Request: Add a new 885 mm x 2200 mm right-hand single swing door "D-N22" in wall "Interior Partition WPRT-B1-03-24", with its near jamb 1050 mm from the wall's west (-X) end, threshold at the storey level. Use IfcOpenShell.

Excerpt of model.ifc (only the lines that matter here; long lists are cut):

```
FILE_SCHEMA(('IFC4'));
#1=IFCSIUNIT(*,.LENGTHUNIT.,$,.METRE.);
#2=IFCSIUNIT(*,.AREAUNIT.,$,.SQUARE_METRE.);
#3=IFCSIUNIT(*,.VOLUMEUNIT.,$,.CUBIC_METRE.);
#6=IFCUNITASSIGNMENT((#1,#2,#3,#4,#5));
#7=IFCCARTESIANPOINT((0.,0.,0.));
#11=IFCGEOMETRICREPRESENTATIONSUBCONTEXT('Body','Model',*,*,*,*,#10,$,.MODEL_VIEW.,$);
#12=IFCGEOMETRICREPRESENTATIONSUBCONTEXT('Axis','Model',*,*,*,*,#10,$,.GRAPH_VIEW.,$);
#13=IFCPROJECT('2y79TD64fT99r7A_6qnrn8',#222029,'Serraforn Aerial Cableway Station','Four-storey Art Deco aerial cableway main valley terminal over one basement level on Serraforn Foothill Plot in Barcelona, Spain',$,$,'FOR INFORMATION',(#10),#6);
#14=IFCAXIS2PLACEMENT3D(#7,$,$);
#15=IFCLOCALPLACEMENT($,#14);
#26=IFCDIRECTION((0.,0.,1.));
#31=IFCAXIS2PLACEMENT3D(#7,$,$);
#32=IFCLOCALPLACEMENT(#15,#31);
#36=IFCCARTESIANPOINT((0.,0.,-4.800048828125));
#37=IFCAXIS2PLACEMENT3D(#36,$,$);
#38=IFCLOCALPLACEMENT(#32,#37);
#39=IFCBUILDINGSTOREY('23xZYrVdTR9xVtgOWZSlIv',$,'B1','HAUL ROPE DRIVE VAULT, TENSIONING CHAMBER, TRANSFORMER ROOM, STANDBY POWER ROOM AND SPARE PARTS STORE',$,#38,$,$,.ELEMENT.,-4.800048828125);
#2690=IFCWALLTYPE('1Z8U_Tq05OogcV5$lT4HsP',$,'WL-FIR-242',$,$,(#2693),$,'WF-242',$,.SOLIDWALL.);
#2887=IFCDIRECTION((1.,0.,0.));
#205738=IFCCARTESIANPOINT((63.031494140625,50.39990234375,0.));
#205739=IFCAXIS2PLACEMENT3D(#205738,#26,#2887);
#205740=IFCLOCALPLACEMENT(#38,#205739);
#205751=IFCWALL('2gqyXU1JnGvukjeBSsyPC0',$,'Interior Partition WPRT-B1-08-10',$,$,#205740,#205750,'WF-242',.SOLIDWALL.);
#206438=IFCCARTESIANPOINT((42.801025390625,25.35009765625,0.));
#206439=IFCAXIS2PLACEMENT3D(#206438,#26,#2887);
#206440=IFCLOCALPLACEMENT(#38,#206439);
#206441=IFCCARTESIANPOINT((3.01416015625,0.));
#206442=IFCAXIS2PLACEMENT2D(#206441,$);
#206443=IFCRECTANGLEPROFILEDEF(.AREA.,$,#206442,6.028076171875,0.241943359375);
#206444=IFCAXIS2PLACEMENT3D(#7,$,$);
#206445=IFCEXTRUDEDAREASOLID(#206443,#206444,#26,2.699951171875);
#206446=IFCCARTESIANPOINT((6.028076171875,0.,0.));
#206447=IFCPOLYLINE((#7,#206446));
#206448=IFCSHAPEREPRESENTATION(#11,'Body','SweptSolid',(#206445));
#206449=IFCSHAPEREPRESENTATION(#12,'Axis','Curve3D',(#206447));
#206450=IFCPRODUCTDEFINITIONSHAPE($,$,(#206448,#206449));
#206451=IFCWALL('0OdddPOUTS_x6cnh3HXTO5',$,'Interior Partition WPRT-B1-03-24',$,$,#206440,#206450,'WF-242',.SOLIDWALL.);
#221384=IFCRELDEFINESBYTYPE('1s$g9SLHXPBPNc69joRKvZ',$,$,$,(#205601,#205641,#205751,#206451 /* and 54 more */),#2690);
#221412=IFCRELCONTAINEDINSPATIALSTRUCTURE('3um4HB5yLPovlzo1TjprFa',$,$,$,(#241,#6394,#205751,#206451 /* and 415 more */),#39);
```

```python
import numpy as np
import ifcopenshell
import ifcopenshell.api.feature
import ifcopenshell.api.geometry
import ifcopenshell.api.root
import ifcopenshell.api.spatial
import ifcopenshell.geom
import ifcopenshell.util.element
import ifcopenshell.util.placement
import ifcopenshell.util.representation
import ifcopenshell.util.shape
import ifcopenshell.util.unit

model = ifcopenshell.open("model.ifc")
unit_scale = ifcopenshell.util.unit.calculate_unit_scale(model)
settings = ifcopenshell.geom.settings()


def volume(element):
    """Net volume in cubic metres, openings subtracted."""
    shape = ifcopenshell.geom.create_shape(settings, element)
    return ifcopenshell.util.shape.get_volume(shape.geometry)


wall = model.by_guid("0OdddPOUTS_x6cnh3HXTO5")
storey = ifcopenshell.util.element.get_container(wall, ifc_class="IfcBuildingStorey")
context = ifcopenshell.util.representation.get_context(model, "Model", "Body", "MODEL_VIEW")
before = volume(wall)

width, height, from_end, sill = 0.885, 2.2, 1.05, 0.0  # metres

# The wall runs along its own X axis, and the end named is its -X end.
wall_shape = ifcopenshell.geom.create_shape(settings, wall)
x, y, z = ifcopenshell.util.shape.get_vertices(wall_shape.geometry).T
start = x.min() + from_end
face, thickness = float(y.min()), float(y.max() - y.min())
wall_matrix = ifcopenshell.util.placement.get_local_placement(wall.ObjectPlacement)
level = ifcopenshell.util.placement.get_local_placement(storey.ObjectPlacement)[2, 3]


def in_wall(x, y):
    """Placement at x, y metres in the wall's axes, at sill height."""
    matrix = wall_matrix.copy()
    matrix[:, 3] = wall_matrix @ np.array([x / unit_scale, y / unit_scale, 0.0, 1.0])
    matrix[2, 3] = level + sill / unit_scale
    return matrix


# Opening: a box that overshoots both wall faces by 50 mm.
opening = ifcopenshell.api.root.create_entity(model, ifc_class="IfcOpeningElement", predefined_type="OPENING")
box = ifcopenshell.api.geometry.add_wall_representation(
    model, context=context, length=width, height=height, thickness=thickness + 0.1
)
ifcopenshell.api.geometry.assign_representation(model, product=opening, representation=box)
ifcopenshell.api.geometry.edit_object_placement(model, product=opening, matrix=in_wall(start, face - 0.05), is_si=False)
ifcopenshell.api.feature.add_feature(model, feature=opening, element=wall)

door = ifcopenshell.api.root.create_entity(model, ifc_class="IfcDoor", name="D-N22", predefined_type="DOOR")
door.OverallWidth, door.OverallHeight = width / unit_scale, height / unit_scale
door.OperationType = "SINGLE_SWING_RIGHT"
body = ifcopenshell.api.geometry.add_door_representation(
    model,
    context=context,
    overall_width=door.OverallWidth,
    overall_height=door.OverallHeight,
    operation_type="SINGLE_SWING_RIGHT",
    lining_properties={"LiningDepth": thickness / unit_scale, "ThresholdDepth": thickness / unit_scale},
)
ifcopenshell.api.geometry.assign_representation(model, product=door, representation=body)
ifcopenshell.api.spatial.assign_container(model, products=[door], relating_structure=storey)
ifcopenshell.api.feature.add_filling(model, opening=opening, element=door)

# The lining spans the wall, so the door starts at the wall face.
ifcopenshell.api.geometry.edit_object_placement(model, product=door, matrix=in_wall(start, face), is_si=False)

after = volume(wall)

print(f"wall volume {before:.3f} -> {after:.3f} m3")

model.write("model_rev.ifc")
```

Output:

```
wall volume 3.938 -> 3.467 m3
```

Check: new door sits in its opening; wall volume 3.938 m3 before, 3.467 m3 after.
